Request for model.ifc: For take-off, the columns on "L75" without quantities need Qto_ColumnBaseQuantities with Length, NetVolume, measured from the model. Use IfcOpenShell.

First a look at what the model holds.

```python
import ifcopenshell
import ifcopenshell.util.element
import ifcopenshell.util.unit

model = ifcopenshell.open("model.ifc")
print(model.schema)
for unit_type in ("LENGTHUNIT", "AREAUNIT", "VOLUMEUNIT"):
    print(unit_type, ifcopenshell.util.unit.calculate_unit_scale(model, unit_type))
storey = next(s for s in model.by_type("IfcBuildingStorey") if s.Name == "L75")
columns = [e for e in ifcopenshell.util.element.get_decomposition(storey) if e.is_a("IfcColumn")]
for e in sorted(columns, key=lambda e: e.id()):
    print(e.id(), e.is_a(), e.Name, list(ifcopenshell.util.element.get_psets(e, qtos_only=True)), sep=" | ")
```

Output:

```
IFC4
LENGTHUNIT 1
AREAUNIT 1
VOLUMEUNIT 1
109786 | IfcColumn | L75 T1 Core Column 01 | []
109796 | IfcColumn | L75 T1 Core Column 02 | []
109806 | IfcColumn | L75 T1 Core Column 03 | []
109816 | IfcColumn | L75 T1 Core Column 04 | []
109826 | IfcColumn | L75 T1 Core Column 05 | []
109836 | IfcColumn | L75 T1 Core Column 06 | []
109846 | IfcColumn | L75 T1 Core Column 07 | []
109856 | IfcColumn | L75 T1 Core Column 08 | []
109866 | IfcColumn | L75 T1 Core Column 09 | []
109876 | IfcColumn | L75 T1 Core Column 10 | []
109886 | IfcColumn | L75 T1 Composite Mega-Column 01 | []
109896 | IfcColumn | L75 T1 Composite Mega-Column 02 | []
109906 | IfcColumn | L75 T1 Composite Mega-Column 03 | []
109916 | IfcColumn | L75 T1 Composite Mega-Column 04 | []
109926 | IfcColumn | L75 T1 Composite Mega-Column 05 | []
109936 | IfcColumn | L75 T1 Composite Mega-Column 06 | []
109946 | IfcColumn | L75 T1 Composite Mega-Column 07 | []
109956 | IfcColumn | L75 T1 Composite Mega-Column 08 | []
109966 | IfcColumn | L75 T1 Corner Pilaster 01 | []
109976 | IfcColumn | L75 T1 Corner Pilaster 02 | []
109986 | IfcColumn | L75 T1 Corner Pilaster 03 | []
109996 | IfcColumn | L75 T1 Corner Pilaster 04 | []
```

```python
import ifcopenshell
import ifcopenshell.api.pset
import ifcopenshell.geom
import ifcopenshell.util.element
import ifcopenshell.util.shape
import ifcopenshell.util.unit

model = ifcopenshell.open("model.ifc")
unit_scale = ifcopenshell.util.unit.calculate_unit_scale(model)
volume_scale = ifcopenshell.util.unit.calculate_unit_scale(model, "VOLUMEUNIT")
settings = ifcopenshell.geom.settings()

storey = next(s for s in model.by_type("IfcBuildingStorey") if s.Name == "L75")
columns = [e for e in ifcopenshell.util.element.get_decomposition(storey) if e.is_a("IfcColumn")]

for e in sorted(columns, key=lambda e: e.id()):
    if ifcopenshell.util.element.get_psets(e, qtos_only=True, should_inherit=False):
        continue
    # Geometry comes back in metres, in the element's own axes.
    shape = ifcopenshell.geom.create_shape(settings, e)
    values = {
        "Length": ifcopenshell.util.shape.get_z(shape.geometry) / unit_scale,
        "NetVolume": ifcopenshell.util.shape.get_volume(shape.geometry) / volume_scale,
    }
    qto = ifcopenshell.api.pset.add_qto(model, product=e, name="Qto_ColumnBaseQuantities")
    ifcopenshell.api.pset.edit_qto(model, qto=qto, properties=values)
    print(e.id(), {k: round(v, 3) for k, v in values.items()})

model.write("model_edited.ifc")
```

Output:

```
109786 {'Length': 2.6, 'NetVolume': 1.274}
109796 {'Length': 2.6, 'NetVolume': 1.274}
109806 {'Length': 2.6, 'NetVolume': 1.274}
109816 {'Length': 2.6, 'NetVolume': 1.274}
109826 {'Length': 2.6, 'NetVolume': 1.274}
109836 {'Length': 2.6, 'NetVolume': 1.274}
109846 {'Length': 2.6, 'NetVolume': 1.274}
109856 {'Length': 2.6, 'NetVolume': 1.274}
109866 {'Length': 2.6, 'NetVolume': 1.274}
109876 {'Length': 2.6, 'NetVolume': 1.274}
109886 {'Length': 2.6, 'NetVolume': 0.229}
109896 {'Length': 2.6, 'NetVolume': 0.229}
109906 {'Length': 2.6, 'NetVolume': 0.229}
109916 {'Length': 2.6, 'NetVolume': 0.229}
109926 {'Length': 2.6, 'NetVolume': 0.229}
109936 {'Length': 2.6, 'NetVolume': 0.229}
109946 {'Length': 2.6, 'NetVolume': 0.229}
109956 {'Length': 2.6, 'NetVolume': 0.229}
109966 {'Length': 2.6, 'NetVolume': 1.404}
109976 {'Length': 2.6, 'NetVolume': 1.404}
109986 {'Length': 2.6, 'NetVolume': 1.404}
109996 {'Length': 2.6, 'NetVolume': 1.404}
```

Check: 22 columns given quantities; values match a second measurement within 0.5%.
